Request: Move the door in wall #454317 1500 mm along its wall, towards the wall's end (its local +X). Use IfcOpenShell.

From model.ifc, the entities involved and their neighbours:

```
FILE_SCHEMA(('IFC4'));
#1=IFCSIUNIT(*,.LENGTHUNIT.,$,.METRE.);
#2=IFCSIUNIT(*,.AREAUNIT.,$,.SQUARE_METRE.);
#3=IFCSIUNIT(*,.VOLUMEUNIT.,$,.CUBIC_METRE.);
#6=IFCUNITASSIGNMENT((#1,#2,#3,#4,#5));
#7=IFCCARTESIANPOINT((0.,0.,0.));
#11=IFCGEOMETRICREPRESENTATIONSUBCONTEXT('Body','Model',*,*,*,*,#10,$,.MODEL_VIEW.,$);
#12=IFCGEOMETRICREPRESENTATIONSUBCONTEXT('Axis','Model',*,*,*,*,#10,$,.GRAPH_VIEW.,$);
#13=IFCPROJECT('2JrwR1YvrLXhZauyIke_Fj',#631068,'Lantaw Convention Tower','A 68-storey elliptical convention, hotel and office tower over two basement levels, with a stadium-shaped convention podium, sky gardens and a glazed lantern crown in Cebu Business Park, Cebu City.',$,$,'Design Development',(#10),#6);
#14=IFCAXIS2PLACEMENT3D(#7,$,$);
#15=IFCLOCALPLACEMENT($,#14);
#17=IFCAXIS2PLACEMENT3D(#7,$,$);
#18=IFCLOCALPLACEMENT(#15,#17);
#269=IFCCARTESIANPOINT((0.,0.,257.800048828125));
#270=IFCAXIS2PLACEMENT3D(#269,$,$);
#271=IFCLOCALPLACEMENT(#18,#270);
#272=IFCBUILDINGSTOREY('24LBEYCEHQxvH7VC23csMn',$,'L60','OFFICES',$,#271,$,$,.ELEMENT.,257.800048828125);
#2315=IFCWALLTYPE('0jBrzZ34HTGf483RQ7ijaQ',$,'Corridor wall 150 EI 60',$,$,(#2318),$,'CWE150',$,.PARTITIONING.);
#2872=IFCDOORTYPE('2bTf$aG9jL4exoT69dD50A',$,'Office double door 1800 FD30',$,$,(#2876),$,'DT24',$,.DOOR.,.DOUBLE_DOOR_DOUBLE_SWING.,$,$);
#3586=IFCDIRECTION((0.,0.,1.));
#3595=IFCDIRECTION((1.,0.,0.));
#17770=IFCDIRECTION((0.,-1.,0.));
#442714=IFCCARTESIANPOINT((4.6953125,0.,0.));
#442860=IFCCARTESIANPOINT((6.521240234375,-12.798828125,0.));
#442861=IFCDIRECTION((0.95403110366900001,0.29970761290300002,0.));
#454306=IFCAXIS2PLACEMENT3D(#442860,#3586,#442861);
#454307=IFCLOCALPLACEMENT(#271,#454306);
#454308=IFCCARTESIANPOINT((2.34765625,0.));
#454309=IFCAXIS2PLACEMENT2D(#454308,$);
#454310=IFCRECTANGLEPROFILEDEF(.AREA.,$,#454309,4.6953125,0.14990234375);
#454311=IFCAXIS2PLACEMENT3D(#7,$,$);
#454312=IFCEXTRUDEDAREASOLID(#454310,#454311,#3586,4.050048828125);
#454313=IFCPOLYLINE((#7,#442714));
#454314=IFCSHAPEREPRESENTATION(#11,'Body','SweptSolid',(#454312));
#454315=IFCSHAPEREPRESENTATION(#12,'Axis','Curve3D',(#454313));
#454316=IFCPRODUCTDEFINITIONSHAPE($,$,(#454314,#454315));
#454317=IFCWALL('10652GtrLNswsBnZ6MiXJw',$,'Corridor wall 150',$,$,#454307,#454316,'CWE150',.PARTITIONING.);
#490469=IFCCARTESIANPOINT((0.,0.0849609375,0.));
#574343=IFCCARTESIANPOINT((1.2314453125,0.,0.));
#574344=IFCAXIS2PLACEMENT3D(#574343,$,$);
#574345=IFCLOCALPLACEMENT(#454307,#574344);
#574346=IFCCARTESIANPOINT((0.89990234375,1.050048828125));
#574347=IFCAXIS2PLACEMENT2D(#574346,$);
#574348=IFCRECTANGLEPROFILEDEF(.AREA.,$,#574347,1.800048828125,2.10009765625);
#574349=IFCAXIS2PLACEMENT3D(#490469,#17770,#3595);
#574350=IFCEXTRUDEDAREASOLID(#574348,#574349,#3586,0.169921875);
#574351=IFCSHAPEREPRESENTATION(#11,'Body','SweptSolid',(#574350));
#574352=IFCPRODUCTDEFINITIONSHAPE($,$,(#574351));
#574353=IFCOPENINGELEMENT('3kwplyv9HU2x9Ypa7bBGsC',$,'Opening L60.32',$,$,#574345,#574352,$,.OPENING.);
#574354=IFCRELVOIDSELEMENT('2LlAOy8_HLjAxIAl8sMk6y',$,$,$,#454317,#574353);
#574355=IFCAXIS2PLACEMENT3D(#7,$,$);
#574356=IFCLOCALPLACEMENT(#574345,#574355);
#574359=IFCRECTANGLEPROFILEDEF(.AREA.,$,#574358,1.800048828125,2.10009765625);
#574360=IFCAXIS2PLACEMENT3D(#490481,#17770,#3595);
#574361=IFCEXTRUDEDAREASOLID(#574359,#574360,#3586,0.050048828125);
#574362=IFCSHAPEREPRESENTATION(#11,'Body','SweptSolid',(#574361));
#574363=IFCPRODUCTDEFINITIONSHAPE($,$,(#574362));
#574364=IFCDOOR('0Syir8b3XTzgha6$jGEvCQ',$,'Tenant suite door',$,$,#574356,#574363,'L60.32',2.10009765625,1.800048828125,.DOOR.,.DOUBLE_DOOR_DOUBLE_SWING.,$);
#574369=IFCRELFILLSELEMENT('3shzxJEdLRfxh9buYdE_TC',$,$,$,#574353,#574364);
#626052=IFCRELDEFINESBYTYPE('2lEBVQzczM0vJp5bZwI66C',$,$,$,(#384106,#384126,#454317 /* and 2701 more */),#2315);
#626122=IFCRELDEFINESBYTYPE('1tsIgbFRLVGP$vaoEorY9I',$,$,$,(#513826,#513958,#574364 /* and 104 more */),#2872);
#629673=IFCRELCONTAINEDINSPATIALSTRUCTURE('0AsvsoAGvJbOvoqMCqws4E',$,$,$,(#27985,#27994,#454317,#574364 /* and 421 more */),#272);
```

```python
import ifcopenshell
import ifcopenshell.api.geometry
import ifcopenshell.util.placement

model = ifcopenshell.open("model.ifc")

door = model.by_guid("0Syir8b3XTzgha6$jGEvCQ")
opening = door.FillsVoids[0].RelatingOpeningElement
wall = opening.VoidsElements[0].RelatingBuildingElement

wall_matrix = ifcopenshell.util.placement.get_local_placement(wall.ObjectPlacement)
shift = wall_matrix[:3, 0] * 1.5
before = ifcopenshell.util.placement.get_local_placement(door.ObjectPlacement)[:3, 3].copy()

# The door is placed relative to its opening, so it follows when the opening moves.
matrix = ifcopenshell.util.placement.get_local_placement(opening.ObjectPlacement)
matrix[:3, 3] += shift
ifcopenshell.api.geometry.edit_object_placement(
    model, product=opening, matrix=matrix, is_si=False, should_transform_children=True
)

after = ifcopenshell.util.placement.get_local_placement(door.ObjectPlacement)[:3, 3]
print("door moved by", (after - before).round(3) + 0.0)

model.write("model-out.ifc")
```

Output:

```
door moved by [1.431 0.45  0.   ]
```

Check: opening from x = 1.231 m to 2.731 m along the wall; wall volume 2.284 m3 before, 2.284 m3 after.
